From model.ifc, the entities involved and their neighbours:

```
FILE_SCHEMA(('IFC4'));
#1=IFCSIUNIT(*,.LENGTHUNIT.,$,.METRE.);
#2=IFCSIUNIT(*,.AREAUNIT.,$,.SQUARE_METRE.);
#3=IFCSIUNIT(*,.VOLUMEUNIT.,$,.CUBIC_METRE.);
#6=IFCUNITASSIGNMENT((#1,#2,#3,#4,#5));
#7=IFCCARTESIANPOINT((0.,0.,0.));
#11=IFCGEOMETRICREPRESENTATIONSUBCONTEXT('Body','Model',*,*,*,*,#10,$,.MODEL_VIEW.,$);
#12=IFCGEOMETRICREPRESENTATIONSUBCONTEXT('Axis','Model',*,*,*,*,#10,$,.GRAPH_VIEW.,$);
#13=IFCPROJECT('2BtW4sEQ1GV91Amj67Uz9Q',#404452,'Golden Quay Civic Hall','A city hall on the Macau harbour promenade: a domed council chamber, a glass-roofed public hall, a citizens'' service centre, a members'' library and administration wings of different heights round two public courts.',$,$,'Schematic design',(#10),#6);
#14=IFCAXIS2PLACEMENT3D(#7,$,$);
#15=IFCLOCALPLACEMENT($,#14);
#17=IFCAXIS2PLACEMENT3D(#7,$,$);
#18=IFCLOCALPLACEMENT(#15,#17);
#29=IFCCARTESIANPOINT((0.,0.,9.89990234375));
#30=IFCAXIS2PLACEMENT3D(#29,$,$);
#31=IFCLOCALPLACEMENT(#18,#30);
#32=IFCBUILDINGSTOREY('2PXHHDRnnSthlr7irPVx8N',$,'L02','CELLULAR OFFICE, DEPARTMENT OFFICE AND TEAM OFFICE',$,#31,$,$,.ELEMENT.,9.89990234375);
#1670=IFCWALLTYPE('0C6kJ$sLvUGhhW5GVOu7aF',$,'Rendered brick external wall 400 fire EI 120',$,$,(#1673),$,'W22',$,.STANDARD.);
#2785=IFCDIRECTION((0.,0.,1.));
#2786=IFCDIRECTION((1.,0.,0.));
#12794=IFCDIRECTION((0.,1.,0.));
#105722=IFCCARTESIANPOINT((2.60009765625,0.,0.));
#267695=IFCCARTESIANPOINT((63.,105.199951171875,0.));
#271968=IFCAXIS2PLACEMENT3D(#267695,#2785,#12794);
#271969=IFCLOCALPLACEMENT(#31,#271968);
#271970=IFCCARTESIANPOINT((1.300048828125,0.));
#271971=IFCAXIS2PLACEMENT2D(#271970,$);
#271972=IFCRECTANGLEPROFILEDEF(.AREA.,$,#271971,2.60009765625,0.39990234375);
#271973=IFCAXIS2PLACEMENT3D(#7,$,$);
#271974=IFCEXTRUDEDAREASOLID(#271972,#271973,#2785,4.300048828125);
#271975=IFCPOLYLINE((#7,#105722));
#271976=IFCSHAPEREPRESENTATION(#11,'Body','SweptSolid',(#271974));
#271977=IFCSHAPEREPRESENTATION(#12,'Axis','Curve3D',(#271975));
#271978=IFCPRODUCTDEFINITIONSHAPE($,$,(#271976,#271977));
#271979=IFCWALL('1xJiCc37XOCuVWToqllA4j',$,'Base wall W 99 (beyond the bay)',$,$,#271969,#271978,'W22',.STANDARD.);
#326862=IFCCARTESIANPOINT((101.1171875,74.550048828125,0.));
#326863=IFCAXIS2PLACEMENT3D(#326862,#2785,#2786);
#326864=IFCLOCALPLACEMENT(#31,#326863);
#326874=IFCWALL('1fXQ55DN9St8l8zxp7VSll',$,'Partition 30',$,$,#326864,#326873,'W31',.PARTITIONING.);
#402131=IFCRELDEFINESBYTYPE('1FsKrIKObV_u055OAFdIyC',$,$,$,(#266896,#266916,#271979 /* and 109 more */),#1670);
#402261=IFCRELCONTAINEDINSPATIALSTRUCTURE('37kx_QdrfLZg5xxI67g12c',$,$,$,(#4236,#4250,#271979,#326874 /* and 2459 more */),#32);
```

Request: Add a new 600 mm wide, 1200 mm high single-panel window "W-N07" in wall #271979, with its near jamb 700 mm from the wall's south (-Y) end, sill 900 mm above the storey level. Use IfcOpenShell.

```python
import numpy as np
import ifcopenshell
import ifcopenshell.api.feature
import ifcopenshell.api.geometry
import ifcopenshell.api.root
import ifcopenshell.api.spatial
import ifcopenshell.geom
import ifcopenshell.util.element
import ifcopenshell.util.placement
import ifcopenshell.util.representation
import ifcopenshell.util.shape
import ifcopenshell.util.unit

model = ifcopenshell.open("model.ifc")
unit_scale = ifcopenshell.util.unit.calculate_unit_scale(model)
settings = ifcopenshell.geom.settings()


def volume(element):
    """Net volume in cubic metres, openings subtracted."""
    shape = ifcopenshell.geom.create_shape(settings, element)
    return ifcopenshell.util.shape.get_volume(shape.geometry)


wall = model.by_guid("1xJiCc37XOCuVWToqllA4j")
storey = ifcopenshell.util.element.get_container(wall, ifc_class="IfcBuildingStorey")
context = ifcopenshell.util.representation.get_context(model, "Model", "Body", "MODEL_VIEW")
before = volume(wall)

width, height, from_end, sill = 0.6, 1.2, 0.7, 0.9  # metres

# The wall runs along its own X axis, and the end named is its -X end.
wall_shape = ifcopenshell.geom.create_shape(settings, wall)
x, y, z = ifcopenshell.util.shape.get_vertices(wall_shape.geometry).T
start = x.min() + from_end
face, thickness = float(y.min()), float(y.max() - y.min())
wall_matrix = ifcopenshell.util.placement.get_local_placement(wall.ObjectPlacement)
level = ifcopenshell.util.placement.get_local_placement(storey.ObjectPlacement)[2, 3]


def in_wall(x, y):
    """Placement at x, y metres in the wall's axes, at sill height."""
    matrix = wall_matrix.copy()
    matrix[:, 3] = wall_matrix @ np.array([x / unit_scale, y / unit_scale, 0.0, 1.0])
    matrix[2, 3] = level + sill / unit_scale
    return matrix


# Opening: a box that overshoots both wall faces by 50 mm.
opening = ifcopenshell.api.root.create_entity(model, ifc_class="IfcOpeningElement", predefined_type="OPENING")
box = ifcopenshell.api.geometry.add_wall_representation(
    model, context=context, length=width, height=height, thickness=thickness + 0.1
)
ifcopenshell.api.geometry.assign_representation(model, product=opening, representation=box)
ifcopenshell.api.geometry.edit_object_placement(model, product=opening, matrix=in_wall(start, face - 0.05), is_si=False)
ifcopenshell.api.feature.add_feature(model, feature=opening, element=wall)

window = ifcopenshell.api.root.create_entity(model, ifc_class="IfcWindow", name="W-N07", predefined_type="WINDOW")
window.OverallWidth, window.OverallHeight = width / unit_scale, height / unit_scale
window.PartitioningType = "SINGLE_PANEL"
body = ifcopenshell.api.geometry.add_window_representation(
    model,
    context=context,
    overall_width=window.OverallWidth,
    overall_height=window.OverallHeight,
    partition_type="SINGLE_PANEL",
)
ifcopenshell.api.geometry.assign_representation(model, product=window, representation=body)
ifcopenshell.api.spatial.assign_container(model, products=[window], relating_structure=storey)
ifcopenshell.api.feature.add_filling(model, opening=opening, element=window)

# Centre the window in the wall's thickness.
ifcopenshell.api.geometry.edit_object_placement(model, product=window, matrix=in_wall(start, face), is_si=False)
window_shape = ifcopenshell.geom.create_shape(settings, window)
depth = ifcopenshell.util.shape.get_vertices(window_shape.geometry)[:, 1]
offset = face + thickness / 2 - (depth.min() + depth.max()) / 2
ifcopenshell.api.geometry.edit_object_placement(model, product=window, matrix=in_wall(start, offset), is_si=False)

after = volume(wall)

print(f"wall volume {before:.3f} -> {after:.3f} m3")

model.write("model_edited.ifc")
```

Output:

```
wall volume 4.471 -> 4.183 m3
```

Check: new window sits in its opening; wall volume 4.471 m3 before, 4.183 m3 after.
